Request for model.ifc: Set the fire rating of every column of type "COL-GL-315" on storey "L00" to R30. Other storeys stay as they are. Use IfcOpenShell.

First a look at what the model holds.

```python
import ifcopenshell
import ifcopenshell.util.element

model = ifcopenshell.open("model.ifc")
print(model.schema)
storey = next(s for s in model.by_type("IfcBuildingStorey") if s.Name == "L00")
columns = [e for e in ifcopenshell.util.element.get_decomposition(storey) if e.is_a("IfcColumn")]
seen = {}
for e in columns:
    element_type = ifcopenshell.util.element.get_type(e)
    key = (element_type.Name if element_type != e and element_type else None, ifcopenshell.util.element.get_pset(e, "Pset_ColumnCommon", "FireRating"))
    seen[key] = seen.get(key, 0) + 1
for (name, value), count in sorted(seen.items(), key=str):
    print(count, "x", name, "|", value)
```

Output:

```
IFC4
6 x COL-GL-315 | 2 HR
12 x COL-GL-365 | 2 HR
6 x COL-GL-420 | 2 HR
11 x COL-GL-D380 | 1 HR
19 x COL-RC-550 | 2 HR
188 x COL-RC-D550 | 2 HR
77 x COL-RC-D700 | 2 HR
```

```python
import ifcopenshell
import ifcopenshell.api.pset
import ifcopenshell.util.element

model = ifcopenshell.open("model.ifc")

storey = next(s for s in model.by_type("IfcBuildingStorey") if s.Name == "L00")
columns = [e for e in ifcopenshell.util.element.get_decomposition(storey) if e.is_a("IfcColumn")]

count = 0
for e in columns:
    element_type = ifcopenshell.util.element.get_type(e)
    if element_type in (None, e) or element_type.Name != "COL-GL-315":
        continue
    # add_pset returns the element's existing set when there is one.
    pset = ifcopenshell.api.pset.add_pset(model, product=e, name="Pset_ColumnCommon")
    ifcopenshell.api.pset.edit_pset(model, pset=pset, properties={"FireRating": "R30"})
    count += 1

print(count, "columns updated")

model.write("model_rev.ifc")
```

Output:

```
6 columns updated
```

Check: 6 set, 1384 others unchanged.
